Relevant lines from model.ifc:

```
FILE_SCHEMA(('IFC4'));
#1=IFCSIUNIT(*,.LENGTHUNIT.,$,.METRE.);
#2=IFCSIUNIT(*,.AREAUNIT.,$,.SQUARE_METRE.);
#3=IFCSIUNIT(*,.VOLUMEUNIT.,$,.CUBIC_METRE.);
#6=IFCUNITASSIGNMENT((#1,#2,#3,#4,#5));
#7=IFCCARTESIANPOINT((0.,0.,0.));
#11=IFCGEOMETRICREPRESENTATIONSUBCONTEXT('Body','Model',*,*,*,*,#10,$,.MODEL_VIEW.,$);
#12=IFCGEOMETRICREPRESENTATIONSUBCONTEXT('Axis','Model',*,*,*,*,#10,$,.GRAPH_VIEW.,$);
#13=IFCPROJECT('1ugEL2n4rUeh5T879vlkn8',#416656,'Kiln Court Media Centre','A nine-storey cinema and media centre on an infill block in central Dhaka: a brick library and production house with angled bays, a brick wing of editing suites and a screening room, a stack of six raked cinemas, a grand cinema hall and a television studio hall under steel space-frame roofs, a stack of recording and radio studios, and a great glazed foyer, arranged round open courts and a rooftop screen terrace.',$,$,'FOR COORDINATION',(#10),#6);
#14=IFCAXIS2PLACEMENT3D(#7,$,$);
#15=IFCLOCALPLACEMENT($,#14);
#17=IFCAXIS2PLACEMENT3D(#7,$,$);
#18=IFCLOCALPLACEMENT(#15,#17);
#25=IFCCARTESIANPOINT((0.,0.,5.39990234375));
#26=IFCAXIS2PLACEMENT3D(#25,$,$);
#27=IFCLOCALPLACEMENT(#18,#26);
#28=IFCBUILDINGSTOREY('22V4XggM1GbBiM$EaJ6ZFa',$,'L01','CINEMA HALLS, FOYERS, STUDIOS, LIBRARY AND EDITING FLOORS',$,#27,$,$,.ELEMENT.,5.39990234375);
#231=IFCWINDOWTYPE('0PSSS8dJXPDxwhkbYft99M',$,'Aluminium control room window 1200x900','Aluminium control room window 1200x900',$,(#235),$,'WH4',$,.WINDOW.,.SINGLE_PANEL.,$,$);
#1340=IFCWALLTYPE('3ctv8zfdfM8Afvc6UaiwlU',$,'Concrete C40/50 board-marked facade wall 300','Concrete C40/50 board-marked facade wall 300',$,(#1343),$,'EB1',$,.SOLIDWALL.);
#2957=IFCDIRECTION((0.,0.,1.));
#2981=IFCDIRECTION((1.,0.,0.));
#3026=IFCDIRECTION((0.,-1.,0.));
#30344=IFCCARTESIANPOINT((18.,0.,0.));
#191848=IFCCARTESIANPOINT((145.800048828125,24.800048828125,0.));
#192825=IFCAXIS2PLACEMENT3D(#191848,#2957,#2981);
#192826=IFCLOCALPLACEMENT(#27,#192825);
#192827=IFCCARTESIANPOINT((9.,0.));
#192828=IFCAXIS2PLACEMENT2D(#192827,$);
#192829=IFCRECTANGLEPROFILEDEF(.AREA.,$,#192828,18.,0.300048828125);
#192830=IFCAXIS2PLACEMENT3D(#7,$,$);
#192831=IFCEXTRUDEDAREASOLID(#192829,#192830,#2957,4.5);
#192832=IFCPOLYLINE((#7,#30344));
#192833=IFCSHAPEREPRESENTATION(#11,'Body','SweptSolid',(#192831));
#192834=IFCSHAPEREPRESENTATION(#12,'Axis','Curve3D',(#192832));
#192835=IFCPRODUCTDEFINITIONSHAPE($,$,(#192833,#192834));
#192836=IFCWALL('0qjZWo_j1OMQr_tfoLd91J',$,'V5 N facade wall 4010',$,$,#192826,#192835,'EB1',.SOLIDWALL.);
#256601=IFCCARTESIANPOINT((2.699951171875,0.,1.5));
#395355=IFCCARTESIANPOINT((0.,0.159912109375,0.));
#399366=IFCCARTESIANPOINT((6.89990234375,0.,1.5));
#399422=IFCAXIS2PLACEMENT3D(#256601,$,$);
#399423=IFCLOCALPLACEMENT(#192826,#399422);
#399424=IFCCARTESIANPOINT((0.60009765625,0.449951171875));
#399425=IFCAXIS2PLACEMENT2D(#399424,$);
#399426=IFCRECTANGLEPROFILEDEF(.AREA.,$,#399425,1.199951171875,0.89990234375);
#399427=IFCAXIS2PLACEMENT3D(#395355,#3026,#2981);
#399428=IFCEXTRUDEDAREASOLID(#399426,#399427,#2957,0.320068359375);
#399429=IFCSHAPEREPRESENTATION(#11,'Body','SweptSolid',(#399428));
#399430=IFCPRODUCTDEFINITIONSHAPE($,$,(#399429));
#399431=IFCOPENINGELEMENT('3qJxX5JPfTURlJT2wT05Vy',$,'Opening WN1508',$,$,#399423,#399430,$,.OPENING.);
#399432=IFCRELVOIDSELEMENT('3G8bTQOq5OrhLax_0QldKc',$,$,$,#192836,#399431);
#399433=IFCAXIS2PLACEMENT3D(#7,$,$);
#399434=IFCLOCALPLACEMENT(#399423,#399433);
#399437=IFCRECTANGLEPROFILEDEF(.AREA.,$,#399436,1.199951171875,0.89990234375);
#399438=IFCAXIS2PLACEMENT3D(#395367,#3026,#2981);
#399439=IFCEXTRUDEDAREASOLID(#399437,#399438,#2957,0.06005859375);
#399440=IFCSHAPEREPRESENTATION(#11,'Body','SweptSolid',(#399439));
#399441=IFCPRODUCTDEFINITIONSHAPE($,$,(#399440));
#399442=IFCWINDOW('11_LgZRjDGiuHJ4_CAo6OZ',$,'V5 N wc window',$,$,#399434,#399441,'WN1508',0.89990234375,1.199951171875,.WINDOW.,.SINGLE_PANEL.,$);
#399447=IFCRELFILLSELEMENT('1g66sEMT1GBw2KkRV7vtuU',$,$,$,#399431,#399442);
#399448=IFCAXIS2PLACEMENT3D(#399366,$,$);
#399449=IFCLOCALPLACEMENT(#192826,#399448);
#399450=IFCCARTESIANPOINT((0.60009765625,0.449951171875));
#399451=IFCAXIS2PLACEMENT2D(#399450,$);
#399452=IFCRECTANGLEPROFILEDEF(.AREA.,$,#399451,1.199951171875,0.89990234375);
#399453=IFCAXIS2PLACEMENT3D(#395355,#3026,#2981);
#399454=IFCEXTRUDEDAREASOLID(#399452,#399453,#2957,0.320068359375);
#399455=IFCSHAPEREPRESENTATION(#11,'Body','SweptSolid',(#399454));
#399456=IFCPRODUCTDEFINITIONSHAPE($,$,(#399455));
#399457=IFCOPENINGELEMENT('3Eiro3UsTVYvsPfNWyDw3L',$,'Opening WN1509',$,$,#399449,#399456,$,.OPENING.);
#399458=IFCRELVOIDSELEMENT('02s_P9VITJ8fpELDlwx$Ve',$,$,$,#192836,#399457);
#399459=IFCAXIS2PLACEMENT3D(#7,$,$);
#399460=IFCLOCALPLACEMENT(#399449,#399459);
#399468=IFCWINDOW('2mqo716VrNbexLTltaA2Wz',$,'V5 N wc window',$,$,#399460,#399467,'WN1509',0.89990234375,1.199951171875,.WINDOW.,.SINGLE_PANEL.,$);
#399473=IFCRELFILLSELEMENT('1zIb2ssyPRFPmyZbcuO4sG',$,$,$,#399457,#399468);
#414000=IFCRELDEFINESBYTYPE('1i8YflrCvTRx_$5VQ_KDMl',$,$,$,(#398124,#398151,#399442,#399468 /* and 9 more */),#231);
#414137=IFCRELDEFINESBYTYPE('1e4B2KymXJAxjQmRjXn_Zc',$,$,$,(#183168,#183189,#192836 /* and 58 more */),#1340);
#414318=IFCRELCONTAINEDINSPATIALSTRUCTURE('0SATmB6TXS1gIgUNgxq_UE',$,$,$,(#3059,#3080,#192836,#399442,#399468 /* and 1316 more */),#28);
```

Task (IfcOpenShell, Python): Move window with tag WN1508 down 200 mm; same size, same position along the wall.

```python
import numpy as np
import ifcopenshell
import ifcopenshell.api.geometry
import ifcopenshell.util.placement
import ifcopenshell.util.unit

model = ifcopenshell.open("model.ifc")
unit_scale = ifcopenshell.util.unit.calculate_unit_scale(model)

window = model.by_guid("11_LgZRjDGiuHJ4_CAo6OZ")
opening = window.FillsVoids[0].RelatingOpeningElement
dz = -0.2

shift = np.array([0.0, 0.0, dz])
# The window is placed relative to its opening, so it follows when the opening moves.
matrix = ifcopenshell.util.placement.get_local_placement(opening.ObjectPlacement)
matrix[:3, 3] += shift
ifcopenshell.api.geometry.edit_object_placement(
    model, product=opening, matrix=matrix, is_si=False, should_transform_children=True
)

print(f"moved by {dz * unit_scale:+.3f} m")

model.write("model-out.ifc")
```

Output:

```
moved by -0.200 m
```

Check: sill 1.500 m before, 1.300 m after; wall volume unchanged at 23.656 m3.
